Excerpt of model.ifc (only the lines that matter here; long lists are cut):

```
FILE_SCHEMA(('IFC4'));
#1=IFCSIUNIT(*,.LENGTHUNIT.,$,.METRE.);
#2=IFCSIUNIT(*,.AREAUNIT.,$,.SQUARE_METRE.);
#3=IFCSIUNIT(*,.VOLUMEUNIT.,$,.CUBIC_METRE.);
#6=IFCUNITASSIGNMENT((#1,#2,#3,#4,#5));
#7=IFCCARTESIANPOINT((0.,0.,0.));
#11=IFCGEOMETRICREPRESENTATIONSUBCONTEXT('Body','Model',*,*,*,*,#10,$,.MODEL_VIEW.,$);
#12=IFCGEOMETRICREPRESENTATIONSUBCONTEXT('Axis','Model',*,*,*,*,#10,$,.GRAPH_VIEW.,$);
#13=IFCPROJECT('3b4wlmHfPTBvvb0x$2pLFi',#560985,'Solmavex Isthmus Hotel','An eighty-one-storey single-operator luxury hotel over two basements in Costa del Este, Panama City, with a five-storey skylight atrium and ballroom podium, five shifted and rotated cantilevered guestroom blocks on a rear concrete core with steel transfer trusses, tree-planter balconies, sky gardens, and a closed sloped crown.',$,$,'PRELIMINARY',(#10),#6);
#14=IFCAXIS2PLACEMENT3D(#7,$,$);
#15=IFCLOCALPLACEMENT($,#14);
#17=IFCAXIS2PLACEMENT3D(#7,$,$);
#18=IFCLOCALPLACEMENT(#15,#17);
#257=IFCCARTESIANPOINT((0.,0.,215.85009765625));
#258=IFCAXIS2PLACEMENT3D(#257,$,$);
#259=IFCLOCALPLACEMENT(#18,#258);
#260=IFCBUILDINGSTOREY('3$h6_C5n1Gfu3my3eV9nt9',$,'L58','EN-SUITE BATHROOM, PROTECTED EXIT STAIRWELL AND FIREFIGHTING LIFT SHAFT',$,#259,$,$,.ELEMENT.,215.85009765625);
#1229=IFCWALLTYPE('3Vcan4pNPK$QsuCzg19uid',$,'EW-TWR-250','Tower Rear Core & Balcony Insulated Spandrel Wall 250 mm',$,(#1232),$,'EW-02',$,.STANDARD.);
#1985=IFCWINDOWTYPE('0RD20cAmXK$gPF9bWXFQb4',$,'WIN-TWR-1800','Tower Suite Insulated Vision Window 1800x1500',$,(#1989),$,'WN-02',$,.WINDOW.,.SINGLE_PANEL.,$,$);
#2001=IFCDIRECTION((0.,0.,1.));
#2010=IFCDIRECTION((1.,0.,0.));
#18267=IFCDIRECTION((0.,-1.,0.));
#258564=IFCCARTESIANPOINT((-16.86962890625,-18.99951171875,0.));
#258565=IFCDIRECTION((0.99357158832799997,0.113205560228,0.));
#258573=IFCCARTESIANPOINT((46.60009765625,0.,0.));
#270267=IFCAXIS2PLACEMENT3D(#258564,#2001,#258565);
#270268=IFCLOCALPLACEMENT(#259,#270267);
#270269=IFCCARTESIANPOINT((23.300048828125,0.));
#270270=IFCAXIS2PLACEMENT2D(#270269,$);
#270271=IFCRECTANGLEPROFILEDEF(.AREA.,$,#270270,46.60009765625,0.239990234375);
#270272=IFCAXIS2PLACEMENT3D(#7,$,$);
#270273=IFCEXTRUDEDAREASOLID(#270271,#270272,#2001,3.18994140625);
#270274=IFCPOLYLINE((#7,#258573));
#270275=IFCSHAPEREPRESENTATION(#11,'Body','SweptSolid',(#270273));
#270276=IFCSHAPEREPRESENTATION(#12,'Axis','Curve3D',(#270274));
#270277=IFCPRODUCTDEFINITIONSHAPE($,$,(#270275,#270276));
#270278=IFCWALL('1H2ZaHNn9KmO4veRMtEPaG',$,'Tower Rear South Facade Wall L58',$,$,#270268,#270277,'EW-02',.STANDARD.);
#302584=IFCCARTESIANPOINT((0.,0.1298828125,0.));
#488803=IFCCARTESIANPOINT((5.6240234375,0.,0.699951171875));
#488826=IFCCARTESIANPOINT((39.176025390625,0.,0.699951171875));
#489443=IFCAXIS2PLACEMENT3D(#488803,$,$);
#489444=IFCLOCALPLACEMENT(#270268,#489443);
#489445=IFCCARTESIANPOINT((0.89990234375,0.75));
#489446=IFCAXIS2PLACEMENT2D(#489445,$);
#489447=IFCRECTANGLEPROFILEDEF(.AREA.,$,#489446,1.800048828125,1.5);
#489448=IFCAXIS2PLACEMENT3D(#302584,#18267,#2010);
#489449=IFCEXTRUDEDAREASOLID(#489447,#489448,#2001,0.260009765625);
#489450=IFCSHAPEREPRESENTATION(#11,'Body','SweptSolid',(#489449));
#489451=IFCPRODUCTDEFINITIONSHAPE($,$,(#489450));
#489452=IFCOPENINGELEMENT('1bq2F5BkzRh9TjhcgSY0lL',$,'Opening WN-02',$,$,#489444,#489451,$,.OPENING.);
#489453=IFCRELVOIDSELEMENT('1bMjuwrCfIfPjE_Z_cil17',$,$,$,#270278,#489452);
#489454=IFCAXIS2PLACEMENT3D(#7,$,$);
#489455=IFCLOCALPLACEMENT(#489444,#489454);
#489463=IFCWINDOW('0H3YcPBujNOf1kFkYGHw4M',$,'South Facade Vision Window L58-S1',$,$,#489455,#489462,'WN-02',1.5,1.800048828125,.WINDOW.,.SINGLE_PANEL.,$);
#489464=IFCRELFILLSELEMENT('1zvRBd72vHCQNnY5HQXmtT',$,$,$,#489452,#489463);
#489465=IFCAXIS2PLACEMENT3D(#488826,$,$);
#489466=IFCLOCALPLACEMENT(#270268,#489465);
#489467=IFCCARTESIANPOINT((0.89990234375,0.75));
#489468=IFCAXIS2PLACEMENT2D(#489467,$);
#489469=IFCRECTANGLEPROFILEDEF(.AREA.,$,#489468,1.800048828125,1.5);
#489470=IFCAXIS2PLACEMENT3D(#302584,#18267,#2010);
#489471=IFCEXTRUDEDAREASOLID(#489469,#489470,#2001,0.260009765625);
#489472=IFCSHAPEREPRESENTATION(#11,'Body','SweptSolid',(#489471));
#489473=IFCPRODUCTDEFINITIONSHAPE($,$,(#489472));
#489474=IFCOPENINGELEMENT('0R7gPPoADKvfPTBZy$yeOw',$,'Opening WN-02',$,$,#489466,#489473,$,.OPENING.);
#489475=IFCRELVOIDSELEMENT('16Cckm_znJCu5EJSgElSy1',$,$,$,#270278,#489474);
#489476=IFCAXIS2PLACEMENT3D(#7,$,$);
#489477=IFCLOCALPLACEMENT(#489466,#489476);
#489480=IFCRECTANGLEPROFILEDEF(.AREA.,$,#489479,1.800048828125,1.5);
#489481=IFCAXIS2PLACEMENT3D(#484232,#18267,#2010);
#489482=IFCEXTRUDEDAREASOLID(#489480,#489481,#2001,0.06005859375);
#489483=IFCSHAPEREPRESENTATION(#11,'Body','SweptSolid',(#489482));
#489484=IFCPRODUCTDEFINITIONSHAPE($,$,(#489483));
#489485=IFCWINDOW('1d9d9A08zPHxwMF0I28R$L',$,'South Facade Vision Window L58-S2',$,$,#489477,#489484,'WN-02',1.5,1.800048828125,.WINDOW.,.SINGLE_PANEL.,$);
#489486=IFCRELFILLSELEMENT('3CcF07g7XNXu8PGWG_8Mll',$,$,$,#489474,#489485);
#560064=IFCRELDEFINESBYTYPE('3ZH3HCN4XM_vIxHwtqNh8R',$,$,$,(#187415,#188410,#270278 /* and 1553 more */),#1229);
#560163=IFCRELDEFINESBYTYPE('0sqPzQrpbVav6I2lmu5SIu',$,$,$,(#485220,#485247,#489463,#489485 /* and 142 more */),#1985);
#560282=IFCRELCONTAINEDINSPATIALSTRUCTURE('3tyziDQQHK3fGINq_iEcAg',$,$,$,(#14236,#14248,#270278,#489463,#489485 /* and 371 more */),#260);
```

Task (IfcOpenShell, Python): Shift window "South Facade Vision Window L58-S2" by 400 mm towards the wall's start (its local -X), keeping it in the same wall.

```python
import ifcopenshell
import ifcopenshell.api.geometry
import ifcopenshell.util.placement
import ifcopenshell.util.unit

model = ifcopenshell.open("model.ifc")
unit_scale = ifcopenshell.util.unit.calculate_unit_scale(model)

window = model.by_guid("1d9d9A08zPHxwMF0I28R$L")
opening = window.FillsVoids[0].RelatingOpeningElement
wall = opening.VoidsElements[0].RelatingBuildingElement

wall_matrix = ifcopenshell.util.placement.get_local_placement(wall.ObjectPlacement)
shift = wall_matrix[:3, 0] * -0.4 / unit_scale
before = ifcopenshell.util.placement.get_local_placement(window.ObjectPlacement)[:3, 3].copy()

# The window is placed relative to its opening, so it follows when the opening moves.
matrix = ifcopenshell.util.placement.get_local_placement(opening.ObjectPlacement)
matrix[:3, 3] += shift
ifcopenshell.api.geometry.edit_object_placement(
    model, product=opening, matrix=matrix, is_si=False, should_transform_children=True
)

after = ifcopenshell.util.placement.get_local_placement(window.ObjectPlacement)[:3, 3]
print("window moved by", (after - before).round(3) + 0.0)

model.write("model_v2.ifc")
```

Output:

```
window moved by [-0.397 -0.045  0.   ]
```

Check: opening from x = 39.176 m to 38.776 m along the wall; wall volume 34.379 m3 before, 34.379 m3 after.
